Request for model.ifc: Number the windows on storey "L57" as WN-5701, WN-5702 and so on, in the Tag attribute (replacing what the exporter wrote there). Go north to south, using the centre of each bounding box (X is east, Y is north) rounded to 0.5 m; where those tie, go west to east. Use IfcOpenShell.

First a look at what the model holds.

```python
import ifcopenshell
import ifcopenshell.util.element
import ifcopenshell.util.placement

model = ifcopenshell.open("model.ifc")
print(model.schema)
storey = next(s for s in model.by_type("IfcBuildingStorey") if s.Name == "L57")
windows = [e for e in ifcopenshell.util.element.get_decomposition(storey) if e.is_a("IfcWindow")]
for e in sorted(windows, key=lambda e: e.id()):
    origin = ifcopenshell.util.placement.get_local_placement(e.ObjectPlacement)[:3, 3]
    print(e.id(), e.Tag, e.Name, origin.round(2) + 0.0, sep=" | ")
```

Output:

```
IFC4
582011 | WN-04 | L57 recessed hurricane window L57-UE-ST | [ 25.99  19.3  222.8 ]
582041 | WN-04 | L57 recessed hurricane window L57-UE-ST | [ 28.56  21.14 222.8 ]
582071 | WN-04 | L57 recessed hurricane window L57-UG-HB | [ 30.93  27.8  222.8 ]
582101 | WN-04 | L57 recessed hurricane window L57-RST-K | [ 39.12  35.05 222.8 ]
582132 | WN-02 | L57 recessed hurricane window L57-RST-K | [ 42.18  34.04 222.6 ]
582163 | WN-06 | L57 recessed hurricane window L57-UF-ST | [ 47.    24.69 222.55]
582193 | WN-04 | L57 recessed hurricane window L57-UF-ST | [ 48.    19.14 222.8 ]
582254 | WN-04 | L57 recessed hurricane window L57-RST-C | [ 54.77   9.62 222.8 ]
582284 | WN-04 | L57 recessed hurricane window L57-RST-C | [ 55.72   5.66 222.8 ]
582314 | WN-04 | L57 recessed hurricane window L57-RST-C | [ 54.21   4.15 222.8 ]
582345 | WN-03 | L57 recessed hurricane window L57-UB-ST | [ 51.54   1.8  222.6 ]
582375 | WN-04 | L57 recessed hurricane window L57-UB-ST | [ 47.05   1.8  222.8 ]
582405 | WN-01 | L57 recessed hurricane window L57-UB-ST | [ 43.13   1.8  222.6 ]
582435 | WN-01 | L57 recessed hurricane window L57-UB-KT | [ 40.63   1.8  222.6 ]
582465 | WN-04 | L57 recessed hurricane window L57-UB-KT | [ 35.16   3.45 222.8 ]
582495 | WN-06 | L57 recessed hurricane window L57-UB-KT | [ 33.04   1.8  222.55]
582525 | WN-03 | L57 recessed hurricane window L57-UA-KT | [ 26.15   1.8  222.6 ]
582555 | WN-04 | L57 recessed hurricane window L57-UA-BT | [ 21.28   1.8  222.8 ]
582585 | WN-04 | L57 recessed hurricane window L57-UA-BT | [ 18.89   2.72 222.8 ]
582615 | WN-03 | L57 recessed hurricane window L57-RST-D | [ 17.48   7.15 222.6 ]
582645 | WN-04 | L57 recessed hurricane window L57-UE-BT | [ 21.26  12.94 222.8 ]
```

```python
import ifcopenshell
import ifcopenshell.geom
import ifcopenshell.util.element
import ifcopenshell.util.shape

model = ifcopenshell.open("model.ifc")
settings = ifcopenshell.geom.settings()
settings.set("use-world-coords", True)


def centre(element):
    shape = ifcopenshell.geom.create_shape(settings, element)
    return ifcopenshell.util.shape.get_bbox_centroid(shape.geometry)


storey = next(s for s in model.by_type("IfcBuildingStorey") if s.Name == "L57")
windows = [e for e in ifcopenshell.util.element.get_decomposition(storey) if e.is_a("IfcWindow")]

# Insertion points can sit at a corner or the storey origin, so sort by the geometry (in metres).
centres = {e: centre(e) for e in windows}
windows.sort(key=lambda e: (-round(centres[e][1] / 0.5), centres[e][0]))

for i, e in enumerate(windows, start=1):
    number = f"WN-57{i:02d}"
    e.Tag = number
    print(e.id(), number)

model.write("model_edited.ifc")
```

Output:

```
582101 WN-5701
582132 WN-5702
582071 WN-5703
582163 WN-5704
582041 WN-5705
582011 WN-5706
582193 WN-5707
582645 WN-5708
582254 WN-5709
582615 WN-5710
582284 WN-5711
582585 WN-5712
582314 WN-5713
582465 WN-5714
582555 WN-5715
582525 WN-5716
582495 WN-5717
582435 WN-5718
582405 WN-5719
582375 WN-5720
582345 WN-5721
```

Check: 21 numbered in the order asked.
